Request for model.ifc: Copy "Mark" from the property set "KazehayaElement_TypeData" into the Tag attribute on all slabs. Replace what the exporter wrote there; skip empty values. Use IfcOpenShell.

First a look at what the model holds.

```python
import ifcopenshell
import ifcopenshell.util.element

model = ifcopenshell.open("model.ifc")
print(model.schema)
slabs = model.by_type("IfcSlab")
print(len(slabs), "slabs")
for e in slabs[:8]:
    source = ifcopenshell.util.element.get_pset(e, "KazehayaElement_TypeData", "Mark")
    target = e.Tag
    print(e.id(), repr(source), repr(target), sep=" | ")
```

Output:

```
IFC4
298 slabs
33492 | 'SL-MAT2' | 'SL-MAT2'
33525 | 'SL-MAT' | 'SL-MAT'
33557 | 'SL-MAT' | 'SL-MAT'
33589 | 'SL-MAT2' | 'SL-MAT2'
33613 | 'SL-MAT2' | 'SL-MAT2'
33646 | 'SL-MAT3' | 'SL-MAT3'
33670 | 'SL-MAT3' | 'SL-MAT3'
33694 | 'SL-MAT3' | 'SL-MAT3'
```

```python
import ifcopenshell
import ifcopenshell.util.element

model = ifcopenshell.open("model.ifc")

count = 0
for e in model.by_type("IfcSlab"):
    value = ifcopenshell.util.element.get_pset(e, "KazehayaElement_TypeData", "Mark")
    current = e.Tag
    if not value or not value.strip() or current == value:
        continue
    e.Tag = value
    count += 1

print(count, "slabs updated")

model.write("model_edited.ifc")
```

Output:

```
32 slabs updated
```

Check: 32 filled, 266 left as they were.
